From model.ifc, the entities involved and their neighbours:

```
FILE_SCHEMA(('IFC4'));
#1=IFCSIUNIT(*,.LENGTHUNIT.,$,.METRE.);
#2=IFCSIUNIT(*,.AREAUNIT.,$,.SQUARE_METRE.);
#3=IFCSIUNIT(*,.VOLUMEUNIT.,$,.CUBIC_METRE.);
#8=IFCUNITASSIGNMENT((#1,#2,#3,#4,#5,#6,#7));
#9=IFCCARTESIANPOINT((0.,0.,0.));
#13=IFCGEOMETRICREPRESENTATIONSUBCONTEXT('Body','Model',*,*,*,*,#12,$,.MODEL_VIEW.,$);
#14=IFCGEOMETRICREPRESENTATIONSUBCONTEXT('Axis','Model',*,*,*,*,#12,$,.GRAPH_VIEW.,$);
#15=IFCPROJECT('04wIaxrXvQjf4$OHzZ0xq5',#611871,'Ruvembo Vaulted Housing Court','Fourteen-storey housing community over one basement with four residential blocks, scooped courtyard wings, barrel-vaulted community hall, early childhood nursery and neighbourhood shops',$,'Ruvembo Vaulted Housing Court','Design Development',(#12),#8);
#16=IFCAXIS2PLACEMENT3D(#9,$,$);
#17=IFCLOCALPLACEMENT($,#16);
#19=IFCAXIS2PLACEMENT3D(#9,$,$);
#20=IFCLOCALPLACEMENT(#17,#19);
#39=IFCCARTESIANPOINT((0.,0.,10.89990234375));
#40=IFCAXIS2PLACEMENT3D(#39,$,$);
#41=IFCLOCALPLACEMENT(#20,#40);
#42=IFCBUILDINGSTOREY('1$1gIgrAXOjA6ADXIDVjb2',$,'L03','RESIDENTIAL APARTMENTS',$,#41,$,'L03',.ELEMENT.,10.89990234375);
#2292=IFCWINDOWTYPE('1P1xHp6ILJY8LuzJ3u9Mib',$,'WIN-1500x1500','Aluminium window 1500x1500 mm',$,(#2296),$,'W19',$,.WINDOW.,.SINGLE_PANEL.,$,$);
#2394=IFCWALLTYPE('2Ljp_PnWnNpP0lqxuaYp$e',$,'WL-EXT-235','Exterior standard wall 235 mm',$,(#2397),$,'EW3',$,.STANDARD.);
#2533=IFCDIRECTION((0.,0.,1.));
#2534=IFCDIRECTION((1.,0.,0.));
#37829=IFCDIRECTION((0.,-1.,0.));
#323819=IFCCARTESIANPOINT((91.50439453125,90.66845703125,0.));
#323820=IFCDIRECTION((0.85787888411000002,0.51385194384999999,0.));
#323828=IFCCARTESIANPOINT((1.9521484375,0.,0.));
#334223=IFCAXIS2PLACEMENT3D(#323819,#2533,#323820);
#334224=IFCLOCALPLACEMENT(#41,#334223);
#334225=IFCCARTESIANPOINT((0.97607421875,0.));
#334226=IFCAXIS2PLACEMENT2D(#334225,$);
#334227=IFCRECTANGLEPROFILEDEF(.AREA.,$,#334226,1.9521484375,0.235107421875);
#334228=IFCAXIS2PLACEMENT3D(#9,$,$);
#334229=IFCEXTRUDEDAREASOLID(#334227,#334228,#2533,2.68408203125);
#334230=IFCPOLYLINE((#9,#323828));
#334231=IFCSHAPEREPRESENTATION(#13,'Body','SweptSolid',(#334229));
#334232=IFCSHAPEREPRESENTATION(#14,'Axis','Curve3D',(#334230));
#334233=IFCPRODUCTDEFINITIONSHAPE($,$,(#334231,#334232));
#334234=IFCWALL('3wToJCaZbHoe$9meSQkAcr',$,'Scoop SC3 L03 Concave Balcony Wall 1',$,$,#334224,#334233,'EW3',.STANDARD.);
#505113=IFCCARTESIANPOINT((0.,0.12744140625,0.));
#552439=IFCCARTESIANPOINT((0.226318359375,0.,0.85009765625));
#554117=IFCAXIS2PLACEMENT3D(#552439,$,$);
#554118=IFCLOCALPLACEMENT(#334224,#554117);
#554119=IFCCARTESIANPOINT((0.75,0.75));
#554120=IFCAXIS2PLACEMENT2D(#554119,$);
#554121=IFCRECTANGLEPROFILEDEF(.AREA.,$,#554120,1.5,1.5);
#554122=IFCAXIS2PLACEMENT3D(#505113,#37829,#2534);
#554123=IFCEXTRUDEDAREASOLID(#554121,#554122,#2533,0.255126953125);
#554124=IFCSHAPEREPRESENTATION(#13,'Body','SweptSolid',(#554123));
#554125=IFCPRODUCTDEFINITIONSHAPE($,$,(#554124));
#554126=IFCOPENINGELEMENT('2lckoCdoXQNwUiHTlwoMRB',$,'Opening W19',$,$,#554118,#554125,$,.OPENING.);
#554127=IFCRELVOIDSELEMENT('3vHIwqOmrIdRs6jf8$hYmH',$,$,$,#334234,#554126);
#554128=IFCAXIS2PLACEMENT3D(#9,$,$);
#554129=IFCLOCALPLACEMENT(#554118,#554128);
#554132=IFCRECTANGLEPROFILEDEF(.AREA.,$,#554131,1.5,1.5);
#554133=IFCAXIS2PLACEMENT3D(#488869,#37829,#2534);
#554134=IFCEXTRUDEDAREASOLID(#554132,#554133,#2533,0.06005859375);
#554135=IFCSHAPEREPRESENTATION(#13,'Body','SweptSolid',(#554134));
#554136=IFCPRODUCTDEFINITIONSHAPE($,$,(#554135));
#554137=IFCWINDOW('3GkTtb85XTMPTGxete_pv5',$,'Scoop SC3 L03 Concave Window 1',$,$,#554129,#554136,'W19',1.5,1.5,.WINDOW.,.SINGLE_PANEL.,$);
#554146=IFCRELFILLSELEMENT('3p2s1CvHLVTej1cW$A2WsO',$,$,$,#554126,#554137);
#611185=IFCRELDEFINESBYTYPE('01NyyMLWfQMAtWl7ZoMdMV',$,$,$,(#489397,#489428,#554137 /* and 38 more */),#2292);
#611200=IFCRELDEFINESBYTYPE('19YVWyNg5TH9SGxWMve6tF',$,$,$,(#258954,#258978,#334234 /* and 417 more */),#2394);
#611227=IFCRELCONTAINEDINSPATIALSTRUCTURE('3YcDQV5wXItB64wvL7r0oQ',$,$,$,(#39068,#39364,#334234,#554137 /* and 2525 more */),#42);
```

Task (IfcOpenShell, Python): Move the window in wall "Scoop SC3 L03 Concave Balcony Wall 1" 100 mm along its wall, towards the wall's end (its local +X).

```python
import ifcopenshell
import ifcopenshell.api.geometry
import ifcopenshell.util.placement
import ifcopenshell.util.unit

model = ifcopenshell.open("model.ifc")
unit_scale = ifcopenshell.util.unit.calculate_unit_scale(model)

window = model.by_guid("3GkTtb85XTMPTGxete_pv5")
opening = window.FillsVoids[0].RelatingOpeningElement
wall = opening.VoidsElements[0].RelatingBuildingElement

wall_matrix = ifcopenshell.util.placement.get_local_placement(wall.ObjectPlacement)
shift = wall_matrix[:3, 0] * 0.1 / unit_scale
before = ifcopenshell.util.placement.get_local_placement(window.ObjectPlacement)[:3, 3].copy()

# The window is placed relative to its opening, so it follows when the opening moves.
matrix = ifcopenshell.util.placement.get_local_placement(opening.ObjectPlacement)
matrix[:3, 3] += shift
ifcopenshell.api.geometry.edit_object_placement(
    model, product=opening, matrix=matrix, is_si=False, should_transform_children=True
)

after = ifcopenshell.util.placement.get_local_placement(window.ObjectPlacement)[:3, 3]
print("window moved by", (after - before).round(3) + 0.0)

model.write("model_updated.ifc")
```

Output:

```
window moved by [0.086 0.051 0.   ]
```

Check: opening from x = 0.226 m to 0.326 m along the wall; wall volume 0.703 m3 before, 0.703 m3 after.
